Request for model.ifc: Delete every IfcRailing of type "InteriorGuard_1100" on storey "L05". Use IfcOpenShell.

First a look at what the model holds.

```python
import ifcopenshell
import ifcopenshell.util.element

model = ifcopenshell.open("model.ifc")
print(model.schema)
storey = next(s for s in model.by_type("IfcBuildingStorey") if s.Name == "L05")
railings = [e for e in ifcopenshell.util.element.get_decomposition(storey) if e.is_a("IfcRailing")]
seen = {}
for e in railings:
    element_type = ifcopenshell.util.element.get_type(e)
    name = element_type.Name if element_type not in (None, e) else None
    seen[name] = seen.get(name, 0) + 1
for name, count in sorted(seen.items(), key=str):
    print(count, "x", name)
```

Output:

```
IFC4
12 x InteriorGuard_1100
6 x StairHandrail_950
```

```python
import ifcopenshell
import ifcopenshell.api.root
import ifcopenshell.util.element

model = ifcopenshell.open("model.ifc")

storey = next(s for s in model.by_type("IfcBuildingStorey") if s.Name == "L05")
railings = [e for e in ifcopenshell.util.element.get_decomposition(storey) if e.is_a("IfcRailing")]
targets = [e for e in railings if (t := ifcopenshell.util.element.get_type(e)) not in (None, e) and t.Name == "InteriorGuard_1100"]

for e in targets:
    ifcopenshell.api.root.remove_product(model, product=e)
print(len(targets), "removed")

model.write("model_updated.ifc")
```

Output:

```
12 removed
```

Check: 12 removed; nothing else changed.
